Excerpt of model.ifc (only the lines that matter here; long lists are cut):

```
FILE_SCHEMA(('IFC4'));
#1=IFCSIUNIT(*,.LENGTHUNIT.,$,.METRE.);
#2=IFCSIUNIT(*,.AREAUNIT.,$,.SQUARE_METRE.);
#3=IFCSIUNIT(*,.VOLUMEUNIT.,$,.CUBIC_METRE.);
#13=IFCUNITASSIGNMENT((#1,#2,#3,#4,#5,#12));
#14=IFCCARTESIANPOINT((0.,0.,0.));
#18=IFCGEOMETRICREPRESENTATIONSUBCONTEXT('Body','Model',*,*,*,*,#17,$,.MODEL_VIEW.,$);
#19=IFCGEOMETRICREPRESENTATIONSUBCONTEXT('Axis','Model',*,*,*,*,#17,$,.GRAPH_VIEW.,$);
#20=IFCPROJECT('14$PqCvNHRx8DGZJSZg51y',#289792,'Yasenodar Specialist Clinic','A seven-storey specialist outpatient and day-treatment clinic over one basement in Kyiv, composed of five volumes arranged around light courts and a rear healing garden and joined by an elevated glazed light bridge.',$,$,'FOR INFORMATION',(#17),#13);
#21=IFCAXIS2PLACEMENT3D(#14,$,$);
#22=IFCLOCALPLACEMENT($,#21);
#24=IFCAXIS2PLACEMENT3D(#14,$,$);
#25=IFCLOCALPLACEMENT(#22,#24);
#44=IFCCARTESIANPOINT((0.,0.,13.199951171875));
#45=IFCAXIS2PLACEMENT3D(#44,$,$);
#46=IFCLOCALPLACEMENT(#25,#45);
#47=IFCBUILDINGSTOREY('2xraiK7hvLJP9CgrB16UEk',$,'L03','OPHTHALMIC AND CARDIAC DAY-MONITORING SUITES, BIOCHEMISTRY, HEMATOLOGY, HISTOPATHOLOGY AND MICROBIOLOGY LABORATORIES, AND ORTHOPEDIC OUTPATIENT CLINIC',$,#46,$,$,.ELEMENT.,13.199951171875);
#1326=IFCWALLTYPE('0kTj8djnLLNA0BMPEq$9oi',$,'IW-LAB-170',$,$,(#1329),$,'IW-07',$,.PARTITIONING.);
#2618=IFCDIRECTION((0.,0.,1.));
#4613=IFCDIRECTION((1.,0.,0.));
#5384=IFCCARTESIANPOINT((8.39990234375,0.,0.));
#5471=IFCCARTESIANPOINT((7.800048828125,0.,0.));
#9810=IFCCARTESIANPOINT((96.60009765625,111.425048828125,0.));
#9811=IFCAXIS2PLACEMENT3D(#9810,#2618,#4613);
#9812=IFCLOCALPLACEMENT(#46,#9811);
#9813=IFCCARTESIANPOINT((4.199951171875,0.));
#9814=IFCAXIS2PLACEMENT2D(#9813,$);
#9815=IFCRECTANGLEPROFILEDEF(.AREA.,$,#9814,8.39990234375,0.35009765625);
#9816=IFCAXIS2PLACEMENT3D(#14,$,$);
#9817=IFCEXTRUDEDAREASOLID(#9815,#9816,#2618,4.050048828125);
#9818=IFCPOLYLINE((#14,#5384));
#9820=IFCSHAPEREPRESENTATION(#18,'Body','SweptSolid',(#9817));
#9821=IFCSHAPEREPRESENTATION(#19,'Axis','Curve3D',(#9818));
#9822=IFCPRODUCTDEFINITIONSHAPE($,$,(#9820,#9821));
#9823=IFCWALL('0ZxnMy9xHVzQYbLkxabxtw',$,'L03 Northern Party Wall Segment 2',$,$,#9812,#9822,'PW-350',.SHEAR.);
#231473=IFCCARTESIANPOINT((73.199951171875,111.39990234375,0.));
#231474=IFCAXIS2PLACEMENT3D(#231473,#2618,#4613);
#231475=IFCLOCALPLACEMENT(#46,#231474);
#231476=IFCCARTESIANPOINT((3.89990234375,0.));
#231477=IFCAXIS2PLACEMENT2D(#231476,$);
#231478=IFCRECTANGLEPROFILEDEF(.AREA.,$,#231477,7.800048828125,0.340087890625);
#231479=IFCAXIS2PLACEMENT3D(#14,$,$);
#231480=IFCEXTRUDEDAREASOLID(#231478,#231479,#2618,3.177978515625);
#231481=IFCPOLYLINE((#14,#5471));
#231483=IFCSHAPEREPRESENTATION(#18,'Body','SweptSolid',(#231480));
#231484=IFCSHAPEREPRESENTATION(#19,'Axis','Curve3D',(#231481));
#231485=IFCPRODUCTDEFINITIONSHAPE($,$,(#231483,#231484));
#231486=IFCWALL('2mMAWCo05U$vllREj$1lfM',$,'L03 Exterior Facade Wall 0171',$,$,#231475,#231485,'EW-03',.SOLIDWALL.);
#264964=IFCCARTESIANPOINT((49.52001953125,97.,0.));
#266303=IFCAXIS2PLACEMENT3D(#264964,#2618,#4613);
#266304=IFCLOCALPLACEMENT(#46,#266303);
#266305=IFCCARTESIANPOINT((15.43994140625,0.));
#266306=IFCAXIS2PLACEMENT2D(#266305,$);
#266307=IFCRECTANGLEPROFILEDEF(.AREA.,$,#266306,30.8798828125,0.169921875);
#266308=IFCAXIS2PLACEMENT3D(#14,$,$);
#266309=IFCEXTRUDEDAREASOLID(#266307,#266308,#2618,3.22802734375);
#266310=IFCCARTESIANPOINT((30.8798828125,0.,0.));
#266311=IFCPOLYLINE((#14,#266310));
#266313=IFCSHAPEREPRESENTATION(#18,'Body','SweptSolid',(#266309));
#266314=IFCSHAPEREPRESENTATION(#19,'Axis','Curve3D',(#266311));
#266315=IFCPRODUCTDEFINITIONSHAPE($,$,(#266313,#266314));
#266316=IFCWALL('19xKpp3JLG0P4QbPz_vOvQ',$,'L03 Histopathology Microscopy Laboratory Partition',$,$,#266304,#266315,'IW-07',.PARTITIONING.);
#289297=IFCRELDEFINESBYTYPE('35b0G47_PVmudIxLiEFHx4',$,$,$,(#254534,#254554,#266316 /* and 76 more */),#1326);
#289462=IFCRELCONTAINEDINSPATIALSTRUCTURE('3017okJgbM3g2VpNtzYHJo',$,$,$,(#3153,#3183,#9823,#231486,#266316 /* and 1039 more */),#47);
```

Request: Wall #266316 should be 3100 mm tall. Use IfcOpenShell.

```python
import ifcopenshell
import ifcopenshell.geom
import ifcopenshell.util.representation
import ifcopenshell.util.shape
import ifcopenshell.util.unit

model = ifcopenshell.open("model.ifc")
unit_scale = ifcopenshell.util.unit.calculate_unit_scale(model)
settings = ifcopenshell.geom.settings()


def volume(element):
    """Net volume in cubic metres, openings subtracted."""
    shape = ifcopenshell.geom.create_shape(settings, element)
    return ifcopenshell.util.shape.get_volume(shape.geometry)


wall = model.by_id(266316)
before = volume(wall)

body = ifcopenshell.util.representation.get_representation(wall, "Model", "Body")
solid = body.Items[0]
old_height = solid.Depth
solid.Depth = 3.1 / unit_scale
after = volume(wall)

print(f"height {old_height:g} -> {solid.Depth:g}, volume {before:.3f} -> {after:.3f} m3")

model.write("model_rev.ifc")
```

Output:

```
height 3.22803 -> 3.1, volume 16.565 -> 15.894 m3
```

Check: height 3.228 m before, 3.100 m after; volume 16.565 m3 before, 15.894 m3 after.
